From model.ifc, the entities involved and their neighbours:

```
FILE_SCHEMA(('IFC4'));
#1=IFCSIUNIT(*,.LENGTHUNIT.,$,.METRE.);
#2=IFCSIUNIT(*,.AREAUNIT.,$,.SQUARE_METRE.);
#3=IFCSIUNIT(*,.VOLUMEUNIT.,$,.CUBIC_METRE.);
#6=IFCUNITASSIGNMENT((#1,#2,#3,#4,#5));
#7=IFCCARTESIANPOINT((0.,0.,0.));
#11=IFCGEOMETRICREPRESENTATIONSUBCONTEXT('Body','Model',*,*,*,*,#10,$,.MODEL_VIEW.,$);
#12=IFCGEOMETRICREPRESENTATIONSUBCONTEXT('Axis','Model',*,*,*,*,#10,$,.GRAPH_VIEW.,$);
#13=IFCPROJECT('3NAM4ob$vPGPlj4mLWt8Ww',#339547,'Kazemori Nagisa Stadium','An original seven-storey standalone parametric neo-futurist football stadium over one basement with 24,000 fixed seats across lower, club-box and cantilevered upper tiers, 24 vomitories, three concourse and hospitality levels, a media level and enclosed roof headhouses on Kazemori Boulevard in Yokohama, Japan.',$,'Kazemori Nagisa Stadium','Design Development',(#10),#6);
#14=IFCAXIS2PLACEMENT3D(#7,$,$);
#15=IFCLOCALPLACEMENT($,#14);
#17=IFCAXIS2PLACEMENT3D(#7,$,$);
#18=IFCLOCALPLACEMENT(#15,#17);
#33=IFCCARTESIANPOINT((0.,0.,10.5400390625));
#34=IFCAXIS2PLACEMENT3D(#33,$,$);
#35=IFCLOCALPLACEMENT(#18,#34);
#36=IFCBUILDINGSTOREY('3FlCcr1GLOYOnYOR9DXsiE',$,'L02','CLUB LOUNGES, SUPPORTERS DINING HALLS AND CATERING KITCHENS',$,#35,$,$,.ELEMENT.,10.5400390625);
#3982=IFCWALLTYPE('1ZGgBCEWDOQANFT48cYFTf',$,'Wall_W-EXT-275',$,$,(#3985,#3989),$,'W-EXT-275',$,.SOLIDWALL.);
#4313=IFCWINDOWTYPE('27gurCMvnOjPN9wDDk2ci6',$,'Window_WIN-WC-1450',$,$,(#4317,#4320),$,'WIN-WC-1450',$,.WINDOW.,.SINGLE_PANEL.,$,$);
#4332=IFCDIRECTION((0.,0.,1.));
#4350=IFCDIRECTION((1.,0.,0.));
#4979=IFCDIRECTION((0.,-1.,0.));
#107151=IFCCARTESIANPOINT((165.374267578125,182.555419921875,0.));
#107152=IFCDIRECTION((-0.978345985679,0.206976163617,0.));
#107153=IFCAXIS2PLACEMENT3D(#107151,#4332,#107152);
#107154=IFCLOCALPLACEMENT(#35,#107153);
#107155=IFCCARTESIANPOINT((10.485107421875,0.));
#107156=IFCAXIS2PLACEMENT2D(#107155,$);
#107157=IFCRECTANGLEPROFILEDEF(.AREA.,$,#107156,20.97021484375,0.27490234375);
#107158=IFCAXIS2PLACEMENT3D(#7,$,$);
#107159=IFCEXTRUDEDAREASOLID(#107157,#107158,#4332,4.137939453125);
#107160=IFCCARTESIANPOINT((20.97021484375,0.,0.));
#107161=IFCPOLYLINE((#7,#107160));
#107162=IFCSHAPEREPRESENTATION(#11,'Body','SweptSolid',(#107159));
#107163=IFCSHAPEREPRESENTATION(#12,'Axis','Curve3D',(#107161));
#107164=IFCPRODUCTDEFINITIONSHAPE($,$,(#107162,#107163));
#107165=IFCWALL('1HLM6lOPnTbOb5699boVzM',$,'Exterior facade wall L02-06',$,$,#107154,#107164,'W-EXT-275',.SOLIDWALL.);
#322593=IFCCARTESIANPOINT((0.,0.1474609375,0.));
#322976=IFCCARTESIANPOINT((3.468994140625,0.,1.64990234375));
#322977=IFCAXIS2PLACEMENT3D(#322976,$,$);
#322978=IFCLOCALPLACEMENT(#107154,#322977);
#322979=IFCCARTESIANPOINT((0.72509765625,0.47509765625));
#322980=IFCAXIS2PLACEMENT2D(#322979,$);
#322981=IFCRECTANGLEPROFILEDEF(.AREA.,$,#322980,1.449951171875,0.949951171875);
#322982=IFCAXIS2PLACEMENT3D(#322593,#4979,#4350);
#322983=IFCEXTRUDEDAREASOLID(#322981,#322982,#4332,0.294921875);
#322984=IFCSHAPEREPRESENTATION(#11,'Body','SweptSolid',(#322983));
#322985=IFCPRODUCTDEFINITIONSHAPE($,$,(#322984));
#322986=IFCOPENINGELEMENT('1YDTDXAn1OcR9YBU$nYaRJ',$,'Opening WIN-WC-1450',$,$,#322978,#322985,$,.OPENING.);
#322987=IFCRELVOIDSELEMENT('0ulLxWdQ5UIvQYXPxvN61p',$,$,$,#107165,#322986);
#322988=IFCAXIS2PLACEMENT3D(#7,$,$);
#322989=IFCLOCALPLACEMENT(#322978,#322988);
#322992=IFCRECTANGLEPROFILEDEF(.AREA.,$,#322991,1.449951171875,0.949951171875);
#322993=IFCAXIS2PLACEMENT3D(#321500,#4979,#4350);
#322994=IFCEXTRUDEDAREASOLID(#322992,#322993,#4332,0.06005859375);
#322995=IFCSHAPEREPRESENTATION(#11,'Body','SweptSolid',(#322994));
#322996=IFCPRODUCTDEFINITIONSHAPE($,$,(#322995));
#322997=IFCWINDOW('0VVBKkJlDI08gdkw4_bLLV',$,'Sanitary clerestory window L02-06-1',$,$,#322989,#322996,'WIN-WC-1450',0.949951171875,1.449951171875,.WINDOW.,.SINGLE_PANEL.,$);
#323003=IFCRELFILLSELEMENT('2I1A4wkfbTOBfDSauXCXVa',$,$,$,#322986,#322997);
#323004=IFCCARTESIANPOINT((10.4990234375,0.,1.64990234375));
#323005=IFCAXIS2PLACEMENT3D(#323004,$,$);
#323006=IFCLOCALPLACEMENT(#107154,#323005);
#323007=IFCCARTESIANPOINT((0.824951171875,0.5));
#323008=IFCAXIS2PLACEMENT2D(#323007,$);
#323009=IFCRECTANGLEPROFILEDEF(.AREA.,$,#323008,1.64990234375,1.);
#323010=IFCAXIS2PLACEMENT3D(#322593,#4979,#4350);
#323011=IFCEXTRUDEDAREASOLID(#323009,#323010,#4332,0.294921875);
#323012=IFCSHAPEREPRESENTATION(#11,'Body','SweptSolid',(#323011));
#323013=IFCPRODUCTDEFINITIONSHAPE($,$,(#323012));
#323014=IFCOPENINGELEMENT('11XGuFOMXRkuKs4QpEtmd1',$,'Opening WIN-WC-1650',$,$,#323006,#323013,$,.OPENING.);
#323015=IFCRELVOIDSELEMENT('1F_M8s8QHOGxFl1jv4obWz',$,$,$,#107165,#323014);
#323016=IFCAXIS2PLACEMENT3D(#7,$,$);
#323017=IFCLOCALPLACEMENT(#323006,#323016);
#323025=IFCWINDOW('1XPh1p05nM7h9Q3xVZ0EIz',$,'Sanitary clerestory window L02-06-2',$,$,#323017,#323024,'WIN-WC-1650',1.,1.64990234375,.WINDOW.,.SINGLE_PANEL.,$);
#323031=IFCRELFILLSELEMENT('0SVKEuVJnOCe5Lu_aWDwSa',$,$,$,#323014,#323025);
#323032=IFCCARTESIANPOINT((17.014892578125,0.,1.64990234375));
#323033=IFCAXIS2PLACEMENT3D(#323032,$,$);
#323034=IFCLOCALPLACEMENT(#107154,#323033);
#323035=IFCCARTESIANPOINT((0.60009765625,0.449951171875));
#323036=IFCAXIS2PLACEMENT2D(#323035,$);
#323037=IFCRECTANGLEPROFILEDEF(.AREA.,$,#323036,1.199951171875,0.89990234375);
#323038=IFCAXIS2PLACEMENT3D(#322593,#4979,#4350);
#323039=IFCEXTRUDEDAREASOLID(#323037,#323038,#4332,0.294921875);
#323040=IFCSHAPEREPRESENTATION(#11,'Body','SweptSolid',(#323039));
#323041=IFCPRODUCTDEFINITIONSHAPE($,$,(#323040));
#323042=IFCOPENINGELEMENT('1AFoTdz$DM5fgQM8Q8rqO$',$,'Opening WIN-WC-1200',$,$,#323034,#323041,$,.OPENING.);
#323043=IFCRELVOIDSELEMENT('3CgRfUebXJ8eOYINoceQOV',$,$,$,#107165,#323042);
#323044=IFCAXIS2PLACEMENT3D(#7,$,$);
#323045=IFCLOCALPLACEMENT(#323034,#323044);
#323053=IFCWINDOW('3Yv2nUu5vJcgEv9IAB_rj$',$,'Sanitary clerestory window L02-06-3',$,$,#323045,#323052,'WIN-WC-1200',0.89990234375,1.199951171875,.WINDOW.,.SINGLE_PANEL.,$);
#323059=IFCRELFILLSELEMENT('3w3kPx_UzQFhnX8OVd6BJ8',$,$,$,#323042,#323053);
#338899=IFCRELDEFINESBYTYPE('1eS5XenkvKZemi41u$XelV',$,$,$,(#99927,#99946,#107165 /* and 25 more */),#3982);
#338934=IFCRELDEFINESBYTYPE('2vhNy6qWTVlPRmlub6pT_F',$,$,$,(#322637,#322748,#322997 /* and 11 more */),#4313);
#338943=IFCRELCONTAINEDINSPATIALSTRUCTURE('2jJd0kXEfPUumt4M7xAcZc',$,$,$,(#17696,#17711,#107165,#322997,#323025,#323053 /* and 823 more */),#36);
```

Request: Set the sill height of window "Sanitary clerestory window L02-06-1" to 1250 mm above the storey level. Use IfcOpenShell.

```python
import numpy as np
import ifcopenshell
import ifcopenshell.api.geometry
import ifcopenshell.geom
import ifcopenshell.util.element
import ifcopenshell.util.placement
import ifcopenshell.util.shape
import ifcopenshell.util.unit

model = ifcopenshell.open("model.ifc")
unit_scale = ifcopenshell.util.unit.calculate_unit_scale(model)

window = model.by_id(322997)
opening = window.FillsVoids[0].RelatingOpeningElement
storey = ifcopenshell.util.element.get_container(window, ifc_class="IfcBuildingStorey")
level = ifcopenshell.util.placement.get_local_placement(storey.ObjectPlacement)[2, 3]

# The opening's origin need not be at the sill, so measure its lowest point.
shape = ifcopenshell.geom.create_shape(ifcopenshell.geom.settings(), opening)
bottom = ifcopenshell.util.shape.get_shape_bottom_elevation(shape, shape.geometry) / unit_scale
dz = level + 1.25 - bottom

shift = np.array([0.0, 0.0, dz])
# The window is placed relative to its opening, so it follows when the opening moves.
matrix = ifcopenshell.util.placement.get_local_placement(opening.ObjectPlacement)
matrix[:3, 3] += shift
ifcopenshell.api.geometry.edit_object_placement(
    model, product=opening, matrix=matrix, is_si=False, should_transform_children=True
)

print(f"moved by {dz * unit_scale:+.3f} m")

model.write("model_updated.ifc")
```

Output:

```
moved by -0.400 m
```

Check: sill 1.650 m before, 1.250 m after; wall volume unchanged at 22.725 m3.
